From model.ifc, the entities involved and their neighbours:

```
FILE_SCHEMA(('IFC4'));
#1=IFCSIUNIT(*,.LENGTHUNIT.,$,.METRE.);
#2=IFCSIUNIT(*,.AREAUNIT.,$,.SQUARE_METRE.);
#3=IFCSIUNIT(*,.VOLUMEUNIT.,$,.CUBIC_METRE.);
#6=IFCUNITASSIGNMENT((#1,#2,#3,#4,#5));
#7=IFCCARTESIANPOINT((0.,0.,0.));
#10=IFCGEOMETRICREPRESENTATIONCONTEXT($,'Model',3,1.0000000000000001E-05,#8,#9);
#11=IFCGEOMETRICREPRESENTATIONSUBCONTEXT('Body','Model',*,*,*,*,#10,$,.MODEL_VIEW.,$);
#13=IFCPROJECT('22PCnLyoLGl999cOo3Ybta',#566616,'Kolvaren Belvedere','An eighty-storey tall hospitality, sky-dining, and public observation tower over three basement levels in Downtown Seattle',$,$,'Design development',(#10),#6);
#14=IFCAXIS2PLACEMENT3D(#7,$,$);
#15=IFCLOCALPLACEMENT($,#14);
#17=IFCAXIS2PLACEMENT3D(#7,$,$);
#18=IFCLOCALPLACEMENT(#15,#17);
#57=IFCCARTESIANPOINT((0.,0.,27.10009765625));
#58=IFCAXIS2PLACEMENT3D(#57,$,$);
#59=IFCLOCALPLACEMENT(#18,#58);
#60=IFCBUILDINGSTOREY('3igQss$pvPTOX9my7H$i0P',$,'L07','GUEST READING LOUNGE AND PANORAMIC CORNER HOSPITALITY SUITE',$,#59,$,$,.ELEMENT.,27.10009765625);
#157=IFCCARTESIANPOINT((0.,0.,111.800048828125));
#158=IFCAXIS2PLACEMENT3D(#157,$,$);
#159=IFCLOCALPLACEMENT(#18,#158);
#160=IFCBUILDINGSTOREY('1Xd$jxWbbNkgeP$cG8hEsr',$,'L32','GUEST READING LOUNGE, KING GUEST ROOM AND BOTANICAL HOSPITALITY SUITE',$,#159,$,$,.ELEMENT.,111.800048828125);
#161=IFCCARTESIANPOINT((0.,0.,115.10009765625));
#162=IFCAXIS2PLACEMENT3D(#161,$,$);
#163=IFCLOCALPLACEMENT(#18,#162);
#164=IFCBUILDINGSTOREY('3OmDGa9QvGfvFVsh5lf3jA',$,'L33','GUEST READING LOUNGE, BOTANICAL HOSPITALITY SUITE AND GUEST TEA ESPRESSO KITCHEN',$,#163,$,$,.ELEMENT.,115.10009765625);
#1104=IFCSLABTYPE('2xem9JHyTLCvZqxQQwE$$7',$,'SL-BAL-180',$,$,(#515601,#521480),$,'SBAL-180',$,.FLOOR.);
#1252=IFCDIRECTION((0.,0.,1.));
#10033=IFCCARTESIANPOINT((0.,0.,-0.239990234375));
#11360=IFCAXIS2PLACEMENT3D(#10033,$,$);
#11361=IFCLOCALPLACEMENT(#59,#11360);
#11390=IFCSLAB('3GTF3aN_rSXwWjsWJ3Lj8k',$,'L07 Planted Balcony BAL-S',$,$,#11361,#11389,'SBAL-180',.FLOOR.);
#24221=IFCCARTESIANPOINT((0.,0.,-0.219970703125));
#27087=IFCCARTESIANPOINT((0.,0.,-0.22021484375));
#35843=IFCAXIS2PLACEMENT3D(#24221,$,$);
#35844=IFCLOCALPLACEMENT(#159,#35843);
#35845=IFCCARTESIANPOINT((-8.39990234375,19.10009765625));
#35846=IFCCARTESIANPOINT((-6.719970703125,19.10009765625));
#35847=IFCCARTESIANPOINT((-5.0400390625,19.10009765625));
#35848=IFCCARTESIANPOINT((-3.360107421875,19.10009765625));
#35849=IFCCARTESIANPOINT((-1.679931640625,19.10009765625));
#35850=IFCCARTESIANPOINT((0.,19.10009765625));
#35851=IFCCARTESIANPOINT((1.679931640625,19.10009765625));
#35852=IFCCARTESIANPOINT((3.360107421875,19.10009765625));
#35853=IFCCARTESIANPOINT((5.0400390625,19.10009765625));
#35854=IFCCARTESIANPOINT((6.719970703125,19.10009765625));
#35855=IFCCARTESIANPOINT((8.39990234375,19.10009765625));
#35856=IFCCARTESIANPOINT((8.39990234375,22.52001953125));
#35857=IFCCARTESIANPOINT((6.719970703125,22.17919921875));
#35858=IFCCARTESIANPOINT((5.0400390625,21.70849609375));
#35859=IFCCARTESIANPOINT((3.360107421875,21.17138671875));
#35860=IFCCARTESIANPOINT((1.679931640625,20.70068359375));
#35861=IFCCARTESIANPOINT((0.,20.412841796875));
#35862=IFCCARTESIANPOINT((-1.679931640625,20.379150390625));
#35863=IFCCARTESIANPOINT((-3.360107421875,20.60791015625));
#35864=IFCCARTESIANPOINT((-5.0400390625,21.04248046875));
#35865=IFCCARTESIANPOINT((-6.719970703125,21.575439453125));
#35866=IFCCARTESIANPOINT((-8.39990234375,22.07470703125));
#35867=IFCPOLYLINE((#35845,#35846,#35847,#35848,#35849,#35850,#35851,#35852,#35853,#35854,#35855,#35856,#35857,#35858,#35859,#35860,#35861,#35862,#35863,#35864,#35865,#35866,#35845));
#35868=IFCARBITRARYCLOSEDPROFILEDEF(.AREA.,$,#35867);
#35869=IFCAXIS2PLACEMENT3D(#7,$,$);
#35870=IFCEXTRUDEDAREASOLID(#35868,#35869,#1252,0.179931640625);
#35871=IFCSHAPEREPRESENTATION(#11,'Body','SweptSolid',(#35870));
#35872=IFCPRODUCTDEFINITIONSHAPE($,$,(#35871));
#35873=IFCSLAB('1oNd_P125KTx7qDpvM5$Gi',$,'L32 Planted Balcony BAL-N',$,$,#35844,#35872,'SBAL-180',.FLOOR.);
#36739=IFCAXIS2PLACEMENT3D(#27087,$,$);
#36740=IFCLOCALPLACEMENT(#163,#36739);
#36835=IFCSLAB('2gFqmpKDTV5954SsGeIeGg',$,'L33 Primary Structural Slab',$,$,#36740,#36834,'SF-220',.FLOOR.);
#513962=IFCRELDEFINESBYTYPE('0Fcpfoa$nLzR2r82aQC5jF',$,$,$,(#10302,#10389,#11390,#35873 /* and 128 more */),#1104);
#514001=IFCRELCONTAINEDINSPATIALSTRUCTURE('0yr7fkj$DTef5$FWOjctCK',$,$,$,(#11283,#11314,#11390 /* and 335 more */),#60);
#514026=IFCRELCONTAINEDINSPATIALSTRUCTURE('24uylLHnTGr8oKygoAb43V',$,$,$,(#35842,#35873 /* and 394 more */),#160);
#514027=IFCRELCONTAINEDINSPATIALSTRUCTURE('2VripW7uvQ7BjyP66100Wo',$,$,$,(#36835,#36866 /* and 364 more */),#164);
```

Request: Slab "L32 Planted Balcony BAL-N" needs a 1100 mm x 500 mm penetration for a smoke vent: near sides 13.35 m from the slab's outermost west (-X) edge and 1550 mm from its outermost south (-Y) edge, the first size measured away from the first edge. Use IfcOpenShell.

```python
import numpy as np
import ifcopenshell
import ifcopenshell.api.feature
import ifcopenshell.api.geometry
import ifcopenshell.api.root
import ifcopenshell.geom
import ifcopenshell.util.placement
import ifcopenshell.util.representation
import ifcopenshell.util.shape
import ifcopenshell.util.unit

model = ifcopenshell.open("model.ifc")
unit_scale = ifcopenshell.util.unit.calculate_unit_scale(model)
settings = ifcopenshell.geom.settings()


def volume(element):
    """Net volume in cubic metres, openings subtracted."""
    shape = ifcopenshell.geom.create_shape(settings, element)
    return ifcopenshell.util.shape.get_volume(shape.geometry)


slab = model.by_guid("1oNd_P125KTx7qDpvM5$Gi")
before = volume(slab)

# Extent in the slab's own axes, in metres. The edges named are its -X and -Y sides.
slab_shape = ifcopenshell.geom.create_shape(settings, slab)
vertices = ifcopenshell.util.shape.get_vertices(slab_shape.geometry)
x_min, y_min, bottom = vertices.min(axis=0)
top = vertices[:, 2].max()

opening = ifcopenshell.api.root.create_entity(model, ifc_class="IfcOpeningElement", name="Smoke vent opening", predefined_type="OPENING")
context = ifcopenshell.util.representation.get_context(model, "Model", "Body", "MODEL_VIEW")
width, depth = 1.1, 0.5
outline = [(0.0, 0.0), (width, 0.0), (width, depth), (0.0, depth), (0.0, 0.0)]
# Overshoot both faces by 50 mm so the cut is clean.
shape = ifcopenshell.api.geometry.add_slab_representation(
    model, context=context, depth=top - bottom + 0.1, polyline=outline
)
ifcopenshell.api.geometry.assign_representation(model, product=opening, representation=shape)

matrix = ifcopenshell.util.placement.get_local_placement(slab.ObjectPlacement)
matrix[:, 3] = matrix @ np.append(np.array([x_min + 13.35, y_min + 1.55, bottom - 0.05]) / unit_scale, 1.0)
ifcopenshell.api.geometry.edit_object_placement(model, product=opening, matrix=matrix, is_si=False)
ifcopenshell.api.feature.add_feature(model, feature=opening, element=slab)

after = volume(slab)

print(f"slab volume {before:.3f} -> {after:.3f} m3")

model.write("model-out.ifc")
```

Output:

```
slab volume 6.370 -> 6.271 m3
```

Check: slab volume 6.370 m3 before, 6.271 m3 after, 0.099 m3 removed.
